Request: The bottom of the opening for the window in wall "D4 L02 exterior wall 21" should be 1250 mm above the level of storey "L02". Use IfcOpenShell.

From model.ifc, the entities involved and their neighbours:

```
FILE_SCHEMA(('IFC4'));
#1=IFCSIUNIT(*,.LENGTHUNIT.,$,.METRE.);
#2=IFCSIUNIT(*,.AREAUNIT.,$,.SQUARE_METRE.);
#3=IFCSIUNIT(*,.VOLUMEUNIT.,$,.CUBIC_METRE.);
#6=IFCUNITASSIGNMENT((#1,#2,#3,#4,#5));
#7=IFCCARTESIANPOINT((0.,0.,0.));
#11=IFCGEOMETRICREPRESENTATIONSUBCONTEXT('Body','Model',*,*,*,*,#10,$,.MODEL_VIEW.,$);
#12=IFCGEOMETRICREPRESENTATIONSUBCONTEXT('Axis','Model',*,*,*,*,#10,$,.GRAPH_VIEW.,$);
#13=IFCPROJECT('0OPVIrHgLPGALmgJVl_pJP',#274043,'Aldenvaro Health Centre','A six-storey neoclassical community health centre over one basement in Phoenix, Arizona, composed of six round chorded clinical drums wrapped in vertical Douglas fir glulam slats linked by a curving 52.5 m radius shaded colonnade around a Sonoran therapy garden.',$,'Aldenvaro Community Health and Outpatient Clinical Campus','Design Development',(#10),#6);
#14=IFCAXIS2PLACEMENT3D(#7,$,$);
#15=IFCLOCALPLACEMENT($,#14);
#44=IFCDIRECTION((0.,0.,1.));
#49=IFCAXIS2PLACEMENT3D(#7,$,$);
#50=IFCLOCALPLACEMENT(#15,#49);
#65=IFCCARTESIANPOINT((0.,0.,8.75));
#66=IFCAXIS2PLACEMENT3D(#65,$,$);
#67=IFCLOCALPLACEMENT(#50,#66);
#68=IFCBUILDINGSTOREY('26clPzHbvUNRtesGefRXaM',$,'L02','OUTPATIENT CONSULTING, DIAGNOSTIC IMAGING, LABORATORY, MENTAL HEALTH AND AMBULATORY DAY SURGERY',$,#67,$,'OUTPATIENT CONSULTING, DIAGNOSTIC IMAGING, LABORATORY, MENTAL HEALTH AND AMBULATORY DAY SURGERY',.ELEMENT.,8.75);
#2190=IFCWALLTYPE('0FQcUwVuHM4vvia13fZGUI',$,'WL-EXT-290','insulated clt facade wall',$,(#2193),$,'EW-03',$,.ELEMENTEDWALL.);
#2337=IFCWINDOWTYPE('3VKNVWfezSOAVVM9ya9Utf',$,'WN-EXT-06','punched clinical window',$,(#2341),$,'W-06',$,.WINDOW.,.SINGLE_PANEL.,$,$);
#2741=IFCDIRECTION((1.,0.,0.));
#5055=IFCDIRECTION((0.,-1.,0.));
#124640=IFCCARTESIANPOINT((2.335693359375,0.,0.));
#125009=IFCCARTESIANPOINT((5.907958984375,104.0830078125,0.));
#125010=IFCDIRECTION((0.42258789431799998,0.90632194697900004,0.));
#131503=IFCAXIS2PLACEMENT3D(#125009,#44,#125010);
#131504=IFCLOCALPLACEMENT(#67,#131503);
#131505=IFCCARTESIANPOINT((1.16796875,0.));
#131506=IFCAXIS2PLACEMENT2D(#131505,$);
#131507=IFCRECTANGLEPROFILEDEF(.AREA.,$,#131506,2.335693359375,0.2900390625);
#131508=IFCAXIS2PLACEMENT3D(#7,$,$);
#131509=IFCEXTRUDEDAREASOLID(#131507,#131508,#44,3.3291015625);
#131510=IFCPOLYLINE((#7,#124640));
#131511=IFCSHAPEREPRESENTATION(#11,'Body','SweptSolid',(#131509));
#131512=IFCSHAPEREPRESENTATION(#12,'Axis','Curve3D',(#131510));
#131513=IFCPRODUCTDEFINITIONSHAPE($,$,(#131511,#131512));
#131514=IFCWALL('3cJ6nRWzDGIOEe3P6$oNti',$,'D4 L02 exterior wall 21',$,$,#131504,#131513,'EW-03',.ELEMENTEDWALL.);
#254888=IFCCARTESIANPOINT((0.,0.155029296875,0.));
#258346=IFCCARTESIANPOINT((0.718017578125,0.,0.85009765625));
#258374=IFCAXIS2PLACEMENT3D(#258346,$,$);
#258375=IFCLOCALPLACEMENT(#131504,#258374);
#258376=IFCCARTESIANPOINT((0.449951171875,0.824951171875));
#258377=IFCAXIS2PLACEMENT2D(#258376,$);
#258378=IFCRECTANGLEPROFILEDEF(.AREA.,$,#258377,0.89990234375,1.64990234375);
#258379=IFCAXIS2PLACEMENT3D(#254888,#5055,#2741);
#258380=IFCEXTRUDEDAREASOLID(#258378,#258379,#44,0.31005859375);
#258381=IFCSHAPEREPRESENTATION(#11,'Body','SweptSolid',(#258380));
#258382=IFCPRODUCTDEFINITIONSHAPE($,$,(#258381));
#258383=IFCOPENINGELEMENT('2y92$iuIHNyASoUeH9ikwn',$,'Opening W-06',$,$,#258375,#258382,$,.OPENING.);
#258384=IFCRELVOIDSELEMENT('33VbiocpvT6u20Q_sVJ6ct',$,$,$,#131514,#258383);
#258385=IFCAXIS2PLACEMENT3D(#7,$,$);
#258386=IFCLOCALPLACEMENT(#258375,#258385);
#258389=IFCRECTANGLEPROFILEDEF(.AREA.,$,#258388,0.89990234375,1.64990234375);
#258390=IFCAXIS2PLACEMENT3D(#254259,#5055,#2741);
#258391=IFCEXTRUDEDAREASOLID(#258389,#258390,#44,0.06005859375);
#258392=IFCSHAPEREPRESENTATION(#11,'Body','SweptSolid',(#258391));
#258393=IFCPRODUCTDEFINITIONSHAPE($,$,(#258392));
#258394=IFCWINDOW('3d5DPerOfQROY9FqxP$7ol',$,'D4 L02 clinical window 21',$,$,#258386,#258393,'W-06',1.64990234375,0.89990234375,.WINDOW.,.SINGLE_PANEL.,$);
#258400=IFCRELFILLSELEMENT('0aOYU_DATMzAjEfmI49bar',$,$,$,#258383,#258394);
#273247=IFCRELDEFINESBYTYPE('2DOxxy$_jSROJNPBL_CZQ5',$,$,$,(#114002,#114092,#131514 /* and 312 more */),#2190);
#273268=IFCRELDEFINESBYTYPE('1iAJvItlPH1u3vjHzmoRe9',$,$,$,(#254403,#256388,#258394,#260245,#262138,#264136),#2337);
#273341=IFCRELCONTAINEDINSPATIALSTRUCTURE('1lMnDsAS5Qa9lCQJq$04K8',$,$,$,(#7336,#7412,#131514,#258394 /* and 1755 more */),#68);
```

```python
import numpy as np
import ifcopenshell
import ifcopenshell.api.geometry
import ifcopenshell.geom
import ifcopenshell.util.element
import ifcopenshell.util.placement
import ifcopenshell.util.shape
import ifcopenshell.util.unit

model = ifcopenshell.open("model.ifc")
unit_scale = ifcopenshell.util.unit.calculate_unit_scale(model)

window = model.by_guid("3d5DPerOfQROY9FqxP$7ol")
opening = window.FillsVoids[0].RelatingOpeningElement
storey = ifcopenshell.util.element.get_container(window, ifc_class="IfcBuildingStorey")
level = ifcopenshell.util.placement.get_local_placement(storey.ObjectPlacement)[2, 3]

# The opening's origin need not be at the sill, so measure its lowest point.
shape = ifcopenshell.geom.create_shape(ifcopenshell.geom.settings(), opening)
bottom = ifcopenshell.util.shape.get_shape_bottom_elevation(shape, shape.geometry) / unit_scale
dz = level + 1.25 - bottom

shift = np.array([0.0, 0.0, dz])
# The window is placed relative to its opening, so it follows when the opening moves.
matrix = ifcopenshell.util.placement.get_local_placement(opening.ObjectPlacement)
matrix[:3, 3] += shift
ifcopenshell.api.geometry.edit_object_placement(
    model, product=opening, matrix=matrix, is_si=False, should_transform_children=True
)

print(f"moved by {dz * unit_scale:+.3f} m")

model.write("model-out.ifc")
```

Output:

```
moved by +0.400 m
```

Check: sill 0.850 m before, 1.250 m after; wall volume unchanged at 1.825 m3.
